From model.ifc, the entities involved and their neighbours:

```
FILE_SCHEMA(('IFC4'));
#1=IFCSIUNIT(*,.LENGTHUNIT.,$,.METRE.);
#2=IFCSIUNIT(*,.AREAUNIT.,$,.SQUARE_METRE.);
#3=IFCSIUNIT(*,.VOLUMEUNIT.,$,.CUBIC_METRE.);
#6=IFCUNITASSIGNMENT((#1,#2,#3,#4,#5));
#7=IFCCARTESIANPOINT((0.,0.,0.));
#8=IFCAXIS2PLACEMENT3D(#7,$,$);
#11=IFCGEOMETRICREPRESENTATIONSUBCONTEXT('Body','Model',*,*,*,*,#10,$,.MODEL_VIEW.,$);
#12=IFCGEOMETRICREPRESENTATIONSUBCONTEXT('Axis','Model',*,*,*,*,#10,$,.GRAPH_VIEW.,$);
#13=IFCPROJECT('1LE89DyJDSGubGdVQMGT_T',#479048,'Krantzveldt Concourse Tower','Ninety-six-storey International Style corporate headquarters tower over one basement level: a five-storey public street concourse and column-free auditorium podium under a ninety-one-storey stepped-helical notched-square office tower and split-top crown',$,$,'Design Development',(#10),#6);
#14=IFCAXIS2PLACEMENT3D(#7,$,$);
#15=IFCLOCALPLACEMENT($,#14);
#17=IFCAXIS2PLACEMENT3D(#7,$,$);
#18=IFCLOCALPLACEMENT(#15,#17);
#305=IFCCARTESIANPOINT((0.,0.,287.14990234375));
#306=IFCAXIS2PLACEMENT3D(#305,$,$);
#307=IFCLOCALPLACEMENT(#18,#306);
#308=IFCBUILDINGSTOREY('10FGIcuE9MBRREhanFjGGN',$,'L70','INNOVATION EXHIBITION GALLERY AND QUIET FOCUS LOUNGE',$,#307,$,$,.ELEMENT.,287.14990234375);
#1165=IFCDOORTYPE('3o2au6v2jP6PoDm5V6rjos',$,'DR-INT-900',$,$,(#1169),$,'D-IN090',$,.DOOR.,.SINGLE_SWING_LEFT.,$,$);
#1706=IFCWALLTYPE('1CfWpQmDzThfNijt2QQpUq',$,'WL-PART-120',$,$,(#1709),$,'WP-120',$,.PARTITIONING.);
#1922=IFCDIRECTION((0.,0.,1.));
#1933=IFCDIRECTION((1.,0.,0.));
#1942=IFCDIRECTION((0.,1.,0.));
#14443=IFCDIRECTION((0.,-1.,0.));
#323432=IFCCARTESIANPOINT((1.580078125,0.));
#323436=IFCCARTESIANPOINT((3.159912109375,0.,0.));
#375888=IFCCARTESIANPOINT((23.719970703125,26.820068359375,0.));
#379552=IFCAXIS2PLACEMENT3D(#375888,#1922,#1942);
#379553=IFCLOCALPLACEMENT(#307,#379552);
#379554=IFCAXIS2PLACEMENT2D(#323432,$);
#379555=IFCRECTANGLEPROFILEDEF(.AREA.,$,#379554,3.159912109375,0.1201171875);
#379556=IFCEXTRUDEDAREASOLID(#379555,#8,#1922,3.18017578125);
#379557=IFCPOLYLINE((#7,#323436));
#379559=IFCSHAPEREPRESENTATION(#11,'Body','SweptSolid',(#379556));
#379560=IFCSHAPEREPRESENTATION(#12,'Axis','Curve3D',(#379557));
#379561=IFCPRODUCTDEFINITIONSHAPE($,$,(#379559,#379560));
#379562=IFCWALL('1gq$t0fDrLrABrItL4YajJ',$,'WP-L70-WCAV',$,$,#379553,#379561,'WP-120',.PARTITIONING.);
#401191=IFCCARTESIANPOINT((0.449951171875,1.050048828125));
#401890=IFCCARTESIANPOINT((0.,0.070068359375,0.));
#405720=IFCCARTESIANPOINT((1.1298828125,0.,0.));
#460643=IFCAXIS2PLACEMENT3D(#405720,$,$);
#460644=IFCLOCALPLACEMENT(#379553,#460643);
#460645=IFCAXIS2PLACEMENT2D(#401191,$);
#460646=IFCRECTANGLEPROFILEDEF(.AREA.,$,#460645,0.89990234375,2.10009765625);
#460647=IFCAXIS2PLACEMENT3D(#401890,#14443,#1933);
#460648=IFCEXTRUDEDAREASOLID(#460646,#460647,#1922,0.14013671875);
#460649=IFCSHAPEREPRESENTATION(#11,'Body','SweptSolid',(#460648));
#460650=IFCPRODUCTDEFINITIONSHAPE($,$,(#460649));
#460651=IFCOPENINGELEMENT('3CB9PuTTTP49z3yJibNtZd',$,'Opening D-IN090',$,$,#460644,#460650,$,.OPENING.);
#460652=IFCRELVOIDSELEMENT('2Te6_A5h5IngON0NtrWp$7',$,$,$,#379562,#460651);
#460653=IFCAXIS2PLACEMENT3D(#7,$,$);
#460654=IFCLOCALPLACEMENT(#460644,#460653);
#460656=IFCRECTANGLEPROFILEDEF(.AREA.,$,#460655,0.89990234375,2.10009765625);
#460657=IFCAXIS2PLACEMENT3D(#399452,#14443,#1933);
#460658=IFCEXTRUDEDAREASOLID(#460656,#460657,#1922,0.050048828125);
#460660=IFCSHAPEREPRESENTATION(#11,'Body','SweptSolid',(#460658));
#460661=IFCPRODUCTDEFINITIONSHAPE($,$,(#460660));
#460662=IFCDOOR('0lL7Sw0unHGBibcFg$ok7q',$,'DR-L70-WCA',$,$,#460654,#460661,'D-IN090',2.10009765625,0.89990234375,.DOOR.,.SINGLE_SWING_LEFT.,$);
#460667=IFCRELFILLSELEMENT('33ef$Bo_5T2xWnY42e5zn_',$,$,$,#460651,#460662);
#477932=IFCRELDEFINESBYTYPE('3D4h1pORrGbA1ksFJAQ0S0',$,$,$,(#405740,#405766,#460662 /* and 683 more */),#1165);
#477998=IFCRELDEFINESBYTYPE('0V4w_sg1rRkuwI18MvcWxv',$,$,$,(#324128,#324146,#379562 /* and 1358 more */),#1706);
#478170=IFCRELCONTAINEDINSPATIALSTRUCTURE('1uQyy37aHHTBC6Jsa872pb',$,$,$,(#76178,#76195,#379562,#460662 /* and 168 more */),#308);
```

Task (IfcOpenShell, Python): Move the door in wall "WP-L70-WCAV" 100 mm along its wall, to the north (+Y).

```python
import ifcopenshell
import ifcopenshell.api.geometry
import ifcopenshell.util.placement

model = ifcopenshell.open("model.ifc")

door = model.by_id(460662)
opening = door.FillsVoids[0].RelatingOpeningElement
wall = opening.VoidsElements[0].RelatingBuildingElement

wall_matrix = ifcopenshell.util.placement.get_local_placement(wall.ObjectPlacement)
shift = wall_matrix[:3, 0] * 0.1
before = ifcopenshell.util.placement.get_local_placement(door.ObjectPlacement)[:3, 3].copy()

# The door is placed relative to its opening, so it follows when the opening moves.
matrix = ifcopenshell.util.placement.get_local_placement(opening.ObjectPlacement)
matrix[:3, 3] += shift
ifcopenshell.api.geometry.edit_object_placement(
    model, product=opening, matrix=matrix, is_si=False, should_transform_children=True
)

after = ifcopenshell.util.placement.get_local_placement(door.ObjectPlacement)[:3, 3]
print("door moved by", (after - before).round(3) + 0.0)

model.write("model_updated.ifc")
```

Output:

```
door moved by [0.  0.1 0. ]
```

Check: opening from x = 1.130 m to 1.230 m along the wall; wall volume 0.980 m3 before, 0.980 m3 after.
